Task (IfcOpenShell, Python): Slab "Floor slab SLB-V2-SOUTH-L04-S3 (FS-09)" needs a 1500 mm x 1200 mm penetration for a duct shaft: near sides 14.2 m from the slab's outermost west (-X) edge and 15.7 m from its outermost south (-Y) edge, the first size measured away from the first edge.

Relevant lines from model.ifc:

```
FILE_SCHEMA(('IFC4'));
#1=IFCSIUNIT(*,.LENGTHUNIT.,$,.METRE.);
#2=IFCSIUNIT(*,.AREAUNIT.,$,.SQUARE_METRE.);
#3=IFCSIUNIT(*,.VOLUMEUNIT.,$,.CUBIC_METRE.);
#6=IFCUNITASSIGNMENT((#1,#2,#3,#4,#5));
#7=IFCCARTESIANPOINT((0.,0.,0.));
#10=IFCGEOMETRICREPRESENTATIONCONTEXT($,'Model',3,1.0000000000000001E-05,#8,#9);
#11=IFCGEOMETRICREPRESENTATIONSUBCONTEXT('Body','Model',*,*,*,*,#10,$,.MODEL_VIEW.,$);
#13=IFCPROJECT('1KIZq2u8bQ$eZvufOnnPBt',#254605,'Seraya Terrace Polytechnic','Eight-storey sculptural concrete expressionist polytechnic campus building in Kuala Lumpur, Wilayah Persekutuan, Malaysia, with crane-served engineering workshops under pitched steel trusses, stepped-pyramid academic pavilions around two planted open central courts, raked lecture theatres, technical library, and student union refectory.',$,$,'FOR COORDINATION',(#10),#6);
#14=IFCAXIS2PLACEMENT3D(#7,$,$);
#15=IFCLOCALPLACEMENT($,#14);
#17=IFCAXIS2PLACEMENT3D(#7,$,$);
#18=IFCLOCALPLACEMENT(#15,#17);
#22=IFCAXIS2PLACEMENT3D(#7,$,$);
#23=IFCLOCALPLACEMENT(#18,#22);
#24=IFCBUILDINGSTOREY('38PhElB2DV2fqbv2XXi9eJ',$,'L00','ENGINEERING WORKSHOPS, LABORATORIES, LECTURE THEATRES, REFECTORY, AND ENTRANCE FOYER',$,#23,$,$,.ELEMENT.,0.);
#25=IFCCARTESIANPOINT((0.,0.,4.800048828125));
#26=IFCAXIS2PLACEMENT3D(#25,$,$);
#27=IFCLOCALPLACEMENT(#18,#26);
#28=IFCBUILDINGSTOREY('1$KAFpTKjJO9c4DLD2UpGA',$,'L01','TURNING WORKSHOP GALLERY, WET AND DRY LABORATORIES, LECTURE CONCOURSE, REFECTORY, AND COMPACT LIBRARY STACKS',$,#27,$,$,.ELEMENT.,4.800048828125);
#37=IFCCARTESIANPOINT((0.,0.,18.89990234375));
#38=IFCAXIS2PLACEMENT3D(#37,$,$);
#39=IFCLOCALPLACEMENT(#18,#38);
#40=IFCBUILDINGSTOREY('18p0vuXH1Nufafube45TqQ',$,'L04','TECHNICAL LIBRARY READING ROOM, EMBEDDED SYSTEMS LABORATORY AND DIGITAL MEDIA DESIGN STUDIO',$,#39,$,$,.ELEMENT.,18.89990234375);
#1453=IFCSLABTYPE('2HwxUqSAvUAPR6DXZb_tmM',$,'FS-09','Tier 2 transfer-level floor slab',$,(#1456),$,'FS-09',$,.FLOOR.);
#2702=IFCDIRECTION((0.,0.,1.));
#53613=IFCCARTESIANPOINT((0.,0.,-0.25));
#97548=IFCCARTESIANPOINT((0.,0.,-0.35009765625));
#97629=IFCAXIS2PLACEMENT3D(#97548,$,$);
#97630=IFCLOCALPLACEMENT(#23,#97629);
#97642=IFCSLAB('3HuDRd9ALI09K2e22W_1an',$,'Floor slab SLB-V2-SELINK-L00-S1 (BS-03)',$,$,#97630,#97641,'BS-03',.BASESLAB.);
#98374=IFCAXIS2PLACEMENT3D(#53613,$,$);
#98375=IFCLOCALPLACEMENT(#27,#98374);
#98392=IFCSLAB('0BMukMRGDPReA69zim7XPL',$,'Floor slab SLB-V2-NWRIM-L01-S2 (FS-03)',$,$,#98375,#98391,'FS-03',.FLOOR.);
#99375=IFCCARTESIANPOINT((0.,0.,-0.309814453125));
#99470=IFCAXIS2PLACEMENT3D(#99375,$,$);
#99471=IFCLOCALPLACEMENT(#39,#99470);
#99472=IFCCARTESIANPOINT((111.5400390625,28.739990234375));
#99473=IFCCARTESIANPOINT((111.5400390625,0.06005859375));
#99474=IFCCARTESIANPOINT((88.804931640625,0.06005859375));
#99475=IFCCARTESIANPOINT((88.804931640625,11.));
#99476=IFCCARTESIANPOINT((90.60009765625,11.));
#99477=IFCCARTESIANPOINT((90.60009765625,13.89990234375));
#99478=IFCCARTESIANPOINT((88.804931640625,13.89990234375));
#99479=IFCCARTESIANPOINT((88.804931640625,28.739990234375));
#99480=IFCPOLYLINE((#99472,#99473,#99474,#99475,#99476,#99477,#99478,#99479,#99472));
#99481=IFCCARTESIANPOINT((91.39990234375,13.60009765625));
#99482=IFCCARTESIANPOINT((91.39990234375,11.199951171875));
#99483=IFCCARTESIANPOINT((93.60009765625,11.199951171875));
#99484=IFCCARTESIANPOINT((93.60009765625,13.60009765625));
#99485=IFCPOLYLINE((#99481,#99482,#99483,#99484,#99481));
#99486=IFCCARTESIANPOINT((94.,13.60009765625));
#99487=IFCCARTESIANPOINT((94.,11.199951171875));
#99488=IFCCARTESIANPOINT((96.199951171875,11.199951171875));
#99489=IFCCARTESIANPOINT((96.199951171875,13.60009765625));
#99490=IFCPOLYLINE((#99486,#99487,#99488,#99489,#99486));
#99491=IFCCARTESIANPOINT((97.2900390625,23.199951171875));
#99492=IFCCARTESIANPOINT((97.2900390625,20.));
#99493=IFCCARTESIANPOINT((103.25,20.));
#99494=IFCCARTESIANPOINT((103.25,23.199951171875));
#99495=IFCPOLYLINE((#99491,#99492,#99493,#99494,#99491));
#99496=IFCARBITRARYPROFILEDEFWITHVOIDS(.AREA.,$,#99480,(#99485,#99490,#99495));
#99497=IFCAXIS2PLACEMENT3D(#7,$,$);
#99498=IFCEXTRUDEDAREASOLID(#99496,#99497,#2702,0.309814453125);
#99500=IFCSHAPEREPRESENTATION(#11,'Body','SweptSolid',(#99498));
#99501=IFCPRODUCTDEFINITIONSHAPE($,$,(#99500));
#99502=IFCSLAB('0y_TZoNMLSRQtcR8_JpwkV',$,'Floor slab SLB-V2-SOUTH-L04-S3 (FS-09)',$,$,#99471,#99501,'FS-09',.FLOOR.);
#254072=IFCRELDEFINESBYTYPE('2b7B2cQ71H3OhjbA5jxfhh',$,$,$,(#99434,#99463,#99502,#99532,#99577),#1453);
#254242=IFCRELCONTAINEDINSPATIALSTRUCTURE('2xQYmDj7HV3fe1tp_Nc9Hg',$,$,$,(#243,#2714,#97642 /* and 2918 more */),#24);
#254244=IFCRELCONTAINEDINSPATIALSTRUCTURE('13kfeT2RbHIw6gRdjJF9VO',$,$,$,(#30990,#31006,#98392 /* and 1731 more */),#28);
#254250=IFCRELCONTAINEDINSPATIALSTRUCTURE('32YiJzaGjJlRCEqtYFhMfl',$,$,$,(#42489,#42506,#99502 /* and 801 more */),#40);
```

```python
import numpy as np
import ifcopenshell
import ifcopenshell.api.feature
import ifcopenshell.api.geometry
import ifcopenshell.api.root
import ifcopenshell.geom
import ifcopenshell.util.placement
import ifcopenshell.util.representation
import ifcopenshell.util.shape
import ifcopenshell.util.unit

model = ifcopenshell.open("model.ifc")
unit_scale = ifcopenshell.util.unit.calculate_unit_scale(model)
settings = ifcopenshell.geom.settings()


def volume(element):
    """Net volume in cubic metres, openings subtracted."""
    shape = ifcopenshell.geom.create_shape(settings, element)
    return ifcopenshell.util.shape.get_volume(shape.geometry)


slab = model.by_id(99502)
before = volume(slab)

# Extent in the slab's own axes, in metres. The edges named are its -X and -Y sides.
slab_shape = ifcopenshell.geom.create_shape(settings, slab)
vertices = ifcopenshell.util.shape.get_vertices(slab_shape.geometry)
x_min, y_min, bottom = vertices.min(axis=0)
top = vertices[:, 2].max()

opening = ifcopenshell.api.root.create_entity(model, ifc_class="IfcOpeningElement", name="Duct shaft opening", predefined_type="OPENING")
context = ifcopenshell.util.representation.get_context(model, "Model", "Body", "MODEL_VIEW")
width, depth = 1.5, 1.2
outline = [(0.0, 0.0), (width, 0.0), (width, depth), (0.0, depth), (0.0, 0.0)]
# Overshoot both faces by 50 mm so the cut is clean.
shape = ifcopenshell.api.geometry.add_slab_representation(
    model, context=context, depth=top - bottom + 0.1, polyline=outline
)
ifcopenshell.api.geometry.assign_representation(model, product=opening, representation=shape)

matrix = ifcopenshell.util.placement.get_local_placement(slab.ObjectPlacement)
matrix[:, 3] = matrix @ np.append(np.array([x_min + 14.2, y_min + 15.7, bottom - 0.05]) / unit_scale, 1.0)
ifcopenshell.api.geometry.edit_object_placement(model, product=opening, matrix=matrix, is_si=False)
ifcopenshell.api.feature.add_feature(model, feature=opening, element=slab)

after = volume(slab)

print(f"slab volume {before:.3f} -> {after:.3f} m3")

model.write("model_edited.ifc")
```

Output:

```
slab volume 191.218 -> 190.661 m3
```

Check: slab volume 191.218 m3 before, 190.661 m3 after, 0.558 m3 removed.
